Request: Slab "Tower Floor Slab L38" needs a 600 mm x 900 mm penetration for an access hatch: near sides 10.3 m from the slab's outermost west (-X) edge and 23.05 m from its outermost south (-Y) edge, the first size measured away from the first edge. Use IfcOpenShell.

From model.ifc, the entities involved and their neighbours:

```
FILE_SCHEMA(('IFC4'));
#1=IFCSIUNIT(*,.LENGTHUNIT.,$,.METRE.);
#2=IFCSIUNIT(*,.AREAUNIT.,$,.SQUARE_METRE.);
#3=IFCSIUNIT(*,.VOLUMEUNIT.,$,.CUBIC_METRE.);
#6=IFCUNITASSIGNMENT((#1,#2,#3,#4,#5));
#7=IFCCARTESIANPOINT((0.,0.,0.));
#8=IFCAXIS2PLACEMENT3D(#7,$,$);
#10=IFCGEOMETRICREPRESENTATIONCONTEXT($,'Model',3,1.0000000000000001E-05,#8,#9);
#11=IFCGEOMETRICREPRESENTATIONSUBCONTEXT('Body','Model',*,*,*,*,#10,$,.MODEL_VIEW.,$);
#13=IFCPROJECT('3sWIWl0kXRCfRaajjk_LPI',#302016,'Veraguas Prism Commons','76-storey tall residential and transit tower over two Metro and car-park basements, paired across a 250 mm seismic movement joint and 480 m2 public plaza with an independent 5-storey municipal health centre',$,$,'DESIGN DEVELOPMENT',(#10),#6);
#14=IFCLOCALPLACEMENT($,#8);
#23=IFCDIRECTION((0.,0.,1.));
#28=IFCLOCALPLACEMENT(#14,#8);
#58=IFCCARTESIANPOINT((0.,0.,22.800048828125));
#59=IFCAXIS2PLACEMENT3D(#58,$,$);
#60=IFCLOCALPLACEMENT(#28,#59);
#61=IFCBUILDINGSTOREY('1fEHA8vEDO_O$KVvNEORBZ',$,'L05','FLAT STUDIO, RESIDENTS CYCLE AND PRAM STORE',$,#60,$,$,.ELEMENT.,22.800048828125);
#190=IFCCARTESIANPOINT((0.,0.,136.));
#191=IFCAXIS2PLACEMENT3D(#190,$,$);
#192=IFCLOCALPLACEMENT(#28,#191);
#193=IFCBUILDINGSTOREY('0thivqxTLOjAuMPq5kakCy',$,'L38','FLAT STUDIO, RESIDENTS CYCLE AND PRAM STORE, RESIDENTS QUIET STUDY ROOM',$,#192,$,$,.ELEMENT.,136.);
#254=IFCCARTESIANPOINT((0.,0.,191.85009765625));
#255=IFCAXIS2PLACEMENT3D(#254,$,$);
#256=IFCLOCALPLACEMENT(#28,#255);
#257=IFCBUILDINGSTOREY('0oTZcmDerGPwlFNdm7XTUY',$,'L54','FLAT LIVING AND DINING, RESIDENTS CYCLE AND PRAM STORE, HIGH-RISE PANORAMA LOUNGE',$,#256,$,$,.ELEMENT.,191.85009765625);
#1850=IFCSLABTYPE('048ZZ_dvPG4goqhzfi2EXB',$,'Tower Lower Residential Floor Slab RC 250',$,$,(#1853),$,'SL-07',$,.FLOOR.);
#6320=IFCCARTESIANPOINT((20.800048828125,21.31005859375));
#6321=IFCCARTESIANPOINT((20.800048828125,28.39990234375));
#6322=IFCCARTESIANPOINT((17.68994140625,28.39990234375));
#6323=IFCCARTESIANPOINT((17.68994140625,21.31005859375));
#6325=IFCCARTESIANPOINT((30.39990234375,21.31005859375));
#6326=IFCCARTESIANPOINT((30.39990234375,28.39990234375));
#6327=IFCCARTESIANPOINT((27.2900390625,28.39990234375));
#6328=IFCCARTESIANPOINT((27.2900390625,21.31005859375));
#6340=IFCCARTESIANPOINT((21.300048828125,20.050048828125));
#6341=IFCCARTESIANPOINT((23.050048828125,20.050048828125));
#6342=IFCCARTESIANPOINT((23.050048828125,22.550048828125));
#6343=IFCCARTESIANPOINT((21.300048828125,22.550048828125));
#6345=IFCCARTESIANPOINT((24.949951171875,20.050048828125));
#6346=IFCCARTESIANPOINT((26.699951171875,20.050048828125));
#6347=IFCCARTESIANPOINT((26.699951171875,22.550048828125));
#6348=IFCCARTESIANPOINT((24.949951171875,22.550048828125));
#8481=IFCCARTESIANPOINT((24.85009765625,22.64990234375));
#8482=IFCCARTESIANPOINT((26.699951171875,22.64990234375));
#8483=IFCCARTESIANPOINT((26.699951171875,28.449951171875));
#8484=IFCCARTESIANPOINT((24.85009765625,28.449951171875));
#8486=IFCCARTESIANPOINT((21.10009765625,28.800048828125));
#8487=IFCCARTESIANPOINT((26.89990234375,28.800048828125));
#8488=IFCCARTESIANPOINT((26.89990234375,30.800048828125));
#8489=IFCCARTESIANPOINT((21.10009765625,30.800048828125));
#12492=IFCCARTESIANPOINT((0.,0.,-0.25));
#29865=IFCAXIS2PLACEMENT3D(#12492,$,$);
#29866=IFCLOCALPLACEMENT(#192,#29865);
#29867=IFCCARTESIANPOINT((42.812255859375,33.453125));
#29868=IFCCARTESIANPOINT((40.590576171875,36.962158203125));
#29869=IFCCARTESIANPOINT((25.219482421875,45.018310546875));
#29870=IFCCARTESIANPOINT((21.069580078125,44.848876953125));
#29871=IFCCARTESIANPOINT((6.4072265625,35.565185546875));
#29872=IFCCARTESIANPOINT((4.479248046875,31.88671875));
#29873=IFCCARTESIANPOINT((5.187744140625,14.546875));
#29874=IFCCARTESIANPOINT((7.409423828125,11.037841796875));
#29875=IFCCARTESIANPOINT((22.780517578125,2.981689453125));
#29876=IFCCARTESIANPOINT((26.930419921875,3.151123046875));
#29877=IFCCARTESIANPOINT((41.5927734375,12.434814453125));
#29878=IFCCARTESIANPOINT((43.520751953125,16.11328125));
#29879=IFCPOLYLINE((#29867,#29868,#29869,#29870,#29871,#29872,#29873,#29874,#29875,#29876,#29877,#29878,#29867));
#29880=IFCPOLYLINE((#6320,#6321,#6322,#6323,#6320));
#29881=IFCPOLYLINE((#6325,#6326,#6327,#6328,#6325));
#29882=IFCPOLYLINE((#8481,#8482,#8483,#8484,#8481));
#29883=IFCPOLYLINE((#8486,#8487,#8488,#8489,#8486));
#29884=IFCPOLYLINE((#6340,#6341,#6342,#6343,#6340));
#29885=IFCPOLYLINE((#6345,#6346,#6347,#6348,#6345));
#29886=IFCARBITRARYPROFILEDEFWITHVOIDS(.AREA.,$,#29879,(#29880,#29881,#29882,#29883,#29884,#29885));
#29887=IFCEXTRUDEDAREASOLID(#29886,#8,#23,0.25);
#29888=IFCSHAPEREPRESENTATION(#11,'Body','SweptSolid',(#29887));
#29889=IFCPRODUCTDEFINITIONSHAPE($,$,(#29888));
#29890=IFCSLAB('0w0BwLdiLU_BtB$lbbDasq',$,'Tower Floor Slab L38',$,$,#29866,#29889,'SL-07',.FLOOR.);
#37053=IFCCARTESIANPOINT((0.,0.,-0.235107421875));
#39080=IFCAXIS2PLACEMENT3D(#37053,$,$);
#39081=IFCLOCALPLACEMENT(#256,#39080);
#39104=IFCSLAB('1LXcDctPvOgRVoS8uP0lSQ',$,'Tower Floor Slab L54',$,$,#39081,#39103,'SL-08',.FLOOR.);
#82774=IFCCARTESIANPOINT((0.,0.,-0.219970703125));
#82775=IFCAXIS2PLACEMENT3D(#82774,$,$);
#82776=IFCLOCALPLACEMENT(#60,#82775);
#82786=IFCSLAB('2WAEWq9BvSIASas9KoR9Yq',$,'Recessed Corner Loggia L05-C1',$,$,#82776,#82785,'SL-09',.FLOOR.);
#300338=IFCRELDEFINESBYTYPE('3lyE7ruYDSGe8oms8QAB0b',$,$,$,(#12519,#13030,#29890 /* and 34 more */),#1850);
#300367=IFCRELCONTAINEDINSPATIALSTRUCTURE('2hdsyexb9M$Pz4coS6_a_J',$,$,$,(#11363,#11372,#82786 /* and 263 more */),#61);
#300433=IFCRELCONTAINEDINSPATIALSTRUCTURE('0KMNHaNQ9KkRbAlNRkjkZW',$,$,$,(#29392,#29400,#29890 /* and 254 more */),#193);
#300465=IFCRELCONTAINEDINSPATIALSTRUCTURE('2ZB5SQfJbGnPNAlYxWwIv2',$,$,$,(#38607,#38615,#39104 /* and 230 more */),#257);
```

```python
import numpy as np
import ifcopenshell
import ifcopenshell.api.feature
import ifcopenshell.api.geometry
import ifcopenshell.api.root
import ifcopenshell.geom
import ifcopenshell.util.placement
import ifcopenshell.util.representation
import ifcopenshell.util.shape
import ifcopenshell.util.unit

model = ifcopenshell.open("model.ifc")
unit_scale = ifcopenshell.util.unit.calculate_unit_scale(model)
settings = ifcopenshell.geom.settings()


def volume(element):
    """Net volume in cubic metres, openings subtracted."""
    shape = ifcopenshell.geom.create_shape(settings, element)
    return ifcopenshell.util.shape.get_volume(shape.geometry)


slab = model.by_guid("0w0BwLdiLU_BtB$lbbDasq")
before = volume(slab)

# Extent in the slab's own axes, in metres. The edges named are its -X and -Y sides.
slab_shape = ifcopenshell.geom.create_shape(settings, slab)
vertices = ifcopenshell.util.shape.get_vertices(slab_shape.geometry)
x_min, y_min, bottom = vertices.min(axis=0)
top = vertices[:, 2].max()

opening = ifcopenshell.api.root.create_entity(model, ifc_class="IfcOpeningElement", name="Access hatch opening", predefined_type="OPENING")
context = ifcopenshell.util.representation.get_context(model, "Model", "Body", "MODEL_VIEW")
width, depth = 0.6, 0.9
outline = [(0.0, 0.0), (width, 0.0), (width, depth), (0.0, depth), (0.0, 0.0)]
# Overshoot both faces by 50 mm so the cut is clean.
shape = ifcopenshell.api.geometry.add_slab_representation(
    model, context=context, depth=top - bottom + 0.1, polyline=outline
)
ifcopenshell.api.geometry.assign_representation(model, product=opening, representation=shape)

matrix = ifcopenshell.util.placement.get_local_placement(slab.ObjectPlacement)
matrix[:, 3] = matrix @ np.append(np.array([x_min + 10.3, y_min + 23.05, bottom - 0.05]) / unit_scale, 1.0)
ifcopenshell.api.geometry.edit_object_placement(model, product=opening, matrix=matrix, is_si=False)
ifcopenshell.api.feature.add_feature(model, feature=opening, element=slab)

after = volume(slab)

print(f"slab volume {before:.3f} -> {after:.3f} m3")

model.write("model_edited.ifc")
```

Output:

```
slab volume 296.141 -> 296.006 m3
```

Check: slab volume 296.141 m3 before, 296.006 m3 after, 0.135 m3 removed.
